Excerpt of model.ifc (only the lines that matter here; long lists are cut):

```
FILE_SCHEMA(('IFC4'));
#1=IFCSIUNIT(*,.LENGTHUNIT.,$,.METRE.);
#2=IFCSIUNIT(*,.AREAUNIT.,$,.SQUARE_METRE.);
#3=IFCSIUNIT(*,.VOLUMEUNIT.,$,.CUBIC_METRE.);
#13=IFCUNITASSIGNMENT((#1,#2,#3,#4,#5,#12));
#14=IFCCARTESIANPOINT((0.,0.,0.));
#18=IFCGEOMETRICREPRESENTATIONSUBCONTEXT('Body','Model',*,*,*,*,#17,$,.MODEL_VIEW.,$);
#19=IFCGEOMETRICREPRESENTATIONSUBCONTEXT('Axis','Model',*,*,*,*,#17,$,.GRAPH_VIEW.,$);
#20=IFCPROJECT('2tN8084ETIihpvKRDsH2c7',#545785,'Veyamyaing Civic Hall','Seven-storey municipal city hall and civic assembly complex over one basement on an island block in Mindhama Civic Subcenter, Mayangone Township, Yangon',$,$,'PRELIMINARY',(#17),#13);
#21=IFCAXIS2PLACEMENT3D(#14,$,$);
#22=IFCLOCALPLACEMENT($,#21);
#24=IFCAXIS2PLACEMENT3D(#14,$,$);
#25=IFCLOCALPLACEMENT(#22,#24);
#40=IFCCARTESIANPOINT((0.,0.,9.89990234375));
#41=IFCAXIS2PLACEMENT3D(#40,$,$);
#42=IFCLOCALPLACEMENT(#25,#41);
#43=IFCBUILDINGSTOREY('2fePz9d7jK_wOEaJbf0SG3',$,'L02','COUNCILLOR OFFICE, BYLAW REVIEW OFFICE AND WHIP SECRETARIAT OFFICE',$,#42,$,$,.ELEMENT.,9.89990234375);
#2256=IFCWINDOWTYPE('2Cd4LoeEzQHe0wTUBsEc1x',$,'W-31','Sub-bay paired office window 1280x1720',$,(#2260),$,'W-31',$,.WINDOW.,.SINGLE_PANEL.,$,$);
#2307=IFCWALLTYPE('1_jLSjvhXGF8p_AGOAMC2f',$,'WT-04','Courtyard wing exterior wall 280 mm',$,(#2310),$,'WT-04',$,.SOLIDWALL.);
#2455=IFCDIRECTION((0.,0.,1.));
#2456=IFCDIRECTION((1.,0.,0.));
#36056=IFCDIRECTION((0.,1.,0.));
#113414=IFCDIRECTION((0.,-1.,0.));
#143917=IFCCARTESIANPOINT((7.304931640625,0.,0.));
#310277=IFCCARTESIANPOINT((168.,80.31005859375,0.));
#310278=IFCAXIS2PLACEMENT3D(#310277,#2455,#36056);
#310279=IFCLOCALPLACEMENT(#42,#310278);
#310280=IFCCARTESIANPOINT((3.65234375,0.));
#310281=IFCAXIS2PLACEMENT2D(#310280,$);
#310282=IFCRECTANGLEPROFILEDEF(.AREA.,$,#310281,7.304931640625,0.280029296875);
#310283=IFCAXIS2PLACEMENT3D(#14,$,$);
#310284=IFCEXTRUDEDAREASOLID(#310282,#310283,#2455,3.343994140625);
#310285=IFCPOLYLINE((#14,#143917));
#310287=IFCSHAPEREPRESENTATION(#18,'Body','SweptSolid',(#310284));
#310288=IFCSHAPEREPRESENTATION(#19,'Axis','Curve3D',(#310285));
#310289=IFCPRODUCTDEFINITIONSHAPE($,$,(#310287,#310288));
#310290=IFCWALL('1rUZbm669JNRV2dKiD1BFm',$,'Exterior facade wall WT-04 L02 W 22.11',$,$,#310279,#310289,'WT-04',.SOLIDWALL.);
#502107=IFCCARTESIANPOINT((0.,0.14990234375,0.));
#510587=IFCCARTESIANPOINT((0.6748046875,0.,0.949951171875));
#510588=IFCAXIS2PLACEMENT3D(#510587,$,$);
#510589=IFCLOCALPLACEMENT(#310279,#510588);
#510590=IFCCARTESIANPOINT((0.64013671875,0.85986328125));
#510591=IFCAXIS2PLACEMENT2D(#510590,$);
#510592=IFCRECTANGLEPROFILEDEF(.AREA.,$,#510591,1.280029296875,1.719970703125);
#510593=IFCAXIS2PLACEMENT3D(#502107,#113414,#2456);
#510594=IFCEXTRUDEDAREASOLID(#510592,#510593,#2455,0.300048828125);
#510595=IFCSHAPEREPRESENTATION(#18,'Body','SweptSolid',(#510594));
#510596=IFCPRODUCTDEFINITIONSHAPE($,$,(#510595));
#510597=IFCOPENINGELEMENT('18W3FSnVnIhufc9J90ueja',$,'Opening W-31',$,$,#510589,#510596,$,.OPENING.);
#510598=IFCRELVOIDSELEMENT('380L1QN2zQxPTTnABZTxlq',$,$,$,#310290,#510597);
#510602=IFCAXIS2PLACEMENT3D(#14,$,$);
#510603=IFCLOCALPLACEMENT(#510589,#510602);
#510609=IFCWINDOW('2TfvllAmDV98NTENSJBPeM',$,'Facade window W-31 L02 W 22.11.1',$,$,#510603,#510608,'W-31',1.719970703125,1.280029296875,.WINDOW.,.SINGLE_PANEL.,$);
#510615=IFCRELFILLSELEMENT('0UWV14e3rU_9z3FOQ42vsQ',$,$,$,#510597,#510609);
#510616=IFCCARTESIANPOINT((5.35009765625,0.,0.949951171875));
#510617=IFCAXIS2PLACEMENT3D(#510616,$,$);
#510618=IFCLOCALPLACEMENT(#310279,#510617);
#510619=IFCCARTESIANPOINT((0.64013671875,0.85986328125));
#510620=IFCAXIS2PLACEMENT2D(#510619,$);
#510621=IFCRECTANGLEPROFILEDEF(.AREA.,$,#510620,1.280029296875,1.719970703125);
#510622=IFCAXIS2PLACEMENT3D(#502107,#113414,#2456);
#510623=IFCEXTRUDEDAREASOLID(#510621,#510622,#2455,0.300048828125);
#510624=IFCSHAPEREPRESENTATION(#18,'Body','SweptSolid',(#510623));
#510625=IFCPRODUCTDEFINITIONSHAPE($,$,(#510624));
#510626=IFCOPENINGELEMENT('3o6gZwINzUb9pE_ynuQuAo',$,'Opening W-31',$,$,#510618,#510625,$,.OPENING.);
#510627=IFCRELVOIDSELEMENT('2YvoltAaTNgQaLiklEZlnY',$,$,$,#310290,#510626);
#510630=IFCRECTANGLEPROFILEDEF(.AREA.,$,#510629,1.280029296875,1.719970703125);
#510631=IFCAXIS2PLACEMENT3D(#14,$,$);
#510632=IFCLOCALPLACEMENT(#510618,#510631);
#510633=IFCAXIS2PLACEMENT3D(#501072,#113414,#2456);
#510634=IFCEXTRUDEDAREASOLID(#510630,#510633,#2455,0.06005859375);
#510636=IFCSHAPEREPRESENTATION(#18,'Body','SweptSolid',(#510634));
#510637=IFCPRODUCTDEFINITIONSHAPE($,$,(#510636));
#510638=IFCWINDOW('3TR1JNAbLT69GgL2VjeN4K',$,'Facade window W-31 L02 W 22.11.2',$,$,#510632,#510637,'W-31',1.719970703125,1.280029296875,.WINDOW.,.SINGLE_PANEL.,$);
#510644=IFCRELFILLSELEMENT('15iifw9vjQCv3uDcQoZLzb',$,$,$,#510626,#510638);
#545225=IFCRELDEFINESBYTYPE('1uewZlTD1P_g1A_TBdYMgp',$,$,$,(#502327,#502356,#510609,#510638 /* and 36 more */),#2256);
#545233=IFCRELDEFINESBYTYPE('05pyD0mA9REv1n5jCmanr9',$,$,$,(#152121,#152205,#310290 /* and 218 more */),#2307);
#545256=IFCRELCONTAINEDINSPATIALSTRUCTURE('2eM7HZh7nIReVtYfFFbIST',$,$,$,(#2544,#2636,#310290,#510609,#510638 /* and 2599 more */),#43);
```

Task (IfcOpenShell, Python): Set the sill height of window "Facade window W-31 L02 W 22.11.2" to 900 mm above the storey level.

```python
import numpy as np
import ifcopenshell
import ifcopenshell.api.geometry
import ifcopenshell.geom
import ifcopenshell.util.element
import ifcopenshell.util.placement
import ifcopenshell.util.shape
import ifcopenshell.util.unit

model = ifcopenshell.open("model.ifc")
unit_scale = ifcopenshell.util.unit.calculate_unit_scale(model)

window = model.by_guid("3TR1JNAbLT69GgL2VjeN4K")
opening = window.FillsVoids[0].RelatingOpeningElement
storey = ifcopenshell.util.element.get_container(window, ifc_class="IfcBuildingStorey")
level = ifcopenshell.util.placement.get_local_placement(storey.ObjectPlacement)[2, 3]

# The opening's origin need not be at the sill, so measure its lowest point.
shape = ifcopenshell.geom.create_shape(ifcopenshell.geom.settings(), opening)
bottom = ifcopenshell.util.shape.get_shape_bottom_elevation(shape, shape.geometry) / unit_scale
dz = level + 0.9 - bottom

shift = np.array([0.0, 0.0, dz])
# The window is placed relative to its opening, so it follows when the opening moves.
matrix = ifcopenshell.util.placement.get_local_placement(opening.ObjectPlacement)
matrix[:3, 3] += shift
ifcopenshell.api.geometry.edit_object_placement(
    model, product=opening, matrix=matrix, is_si=False, should_transform_children=True
)

print(f"moved by {dz * unit_scale:+.3f} m")

model.write("model_v2.ifc")
```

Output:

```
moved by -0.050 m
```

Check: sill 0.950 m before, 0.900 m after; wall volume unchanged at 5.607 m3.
